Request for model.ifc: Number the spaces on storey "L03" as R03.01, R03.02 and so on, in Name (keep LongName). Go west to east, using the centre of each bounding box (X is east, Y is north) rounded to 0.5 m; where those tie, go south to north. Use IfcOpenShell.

First a look at what the model holds.

```python
import ifcopenshell
import ifcopenshell.util.element
import ifcopenshell.util.placement

model = ifcopenshell.open("model.ifc")
print(model.schema)
storey = next(s for s in model.by_type("IfcBuildingStorey") if s.Name == "L03")
spaces = [e for e in ifcopenshell.util.element.get_decomposition(storey) if e.is_a("IfcSpace")]
for e in sorted(spaces, key=lambda e: e.id()):
    origin = ifcopenshell.util.placement.get_local_placement(e.ObjectPlacement)[:3, 3]
    print(e.id(), e.Name, e.LongName, origin.round(2) + 0.0, sep=" | ")
```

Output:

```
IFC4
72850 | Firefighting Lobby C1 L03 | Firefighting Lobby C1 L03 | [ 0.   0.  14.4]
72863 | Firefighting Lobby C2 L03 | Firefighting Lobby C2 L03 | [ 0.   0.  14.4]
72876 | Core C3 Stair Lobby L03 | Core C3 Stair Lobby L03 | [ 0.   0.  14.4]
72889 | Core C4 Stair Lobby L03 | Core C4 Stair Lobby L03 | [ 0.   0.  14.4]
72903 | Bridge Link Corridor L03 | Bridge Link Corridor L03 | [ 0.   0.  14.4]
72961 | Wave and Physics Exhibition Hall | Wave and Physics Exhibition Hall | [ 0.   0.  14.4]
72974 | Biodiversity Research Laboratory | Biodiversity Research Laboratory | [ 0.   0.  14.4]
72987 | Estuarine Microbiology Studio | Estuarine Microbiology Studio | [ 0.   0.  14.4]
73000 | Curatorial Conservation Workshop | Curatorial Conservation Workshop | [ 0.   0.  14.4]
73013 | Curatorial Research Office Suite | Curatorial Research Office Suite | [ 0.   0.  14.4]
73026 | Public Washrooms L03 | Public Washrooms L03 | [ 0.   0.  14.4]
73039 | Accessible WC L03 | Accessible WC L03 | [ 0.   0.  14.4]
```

```python
import ifcopenshell
import ifcopenshell.geom
import ifcopenshell.util.element
import ifcopenshell.util.shape

model = ifcopenshell.open("model.ifc")
settings = ifcopenshell.geom.settings()
settings.set("use-world-coords", True)


def centre(element):
    shape = ifcopenshell.geom.create_shape(settings, element)
    return ifcopenshell.util.shape.get_bbox_centroid(shape.geometry)


storey = next(s for s in model.by_type("IfcBuildingStorey") if s.Name == "L03")
spaces = [e for e in ifcopenshell.util.element.get_decomposition(storey) if e.is_a("IfcSpace")]

# Insertion points can sit at a corner or the storey origin, so sort by the geometry (in metres).
centres = {e: centre(e) for e in spaces}
spaces.sort(key=lambda e: (round(centres[e][0] / 0.5), centres[e][1]))

for i, e in enumerate(spaces, start=1):
    number = f"R03.{i:02d}"
    e.Name = number
    print(e.id(), number)

model.write("model-out.ifc")
```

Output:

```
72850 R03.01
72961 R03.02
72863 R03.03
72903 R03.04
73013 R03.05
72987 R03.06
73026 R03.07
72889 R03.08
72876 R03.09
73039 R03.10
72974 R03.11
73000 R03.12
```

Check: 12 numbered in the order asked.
